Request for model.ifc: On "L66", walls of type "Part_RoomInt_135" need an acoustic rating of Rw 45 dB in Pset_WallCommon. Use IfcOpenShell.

First a look at what the model holds.

```python
import ifcopenshell
import ifcopenshell.util.element

model = ifcopenshell.open("model.ifc")
print(model.schema)
storey = next(s for s in model.by_type("IfcBuildingStorey") if s.Name == "L66")
walls = [e for e in ifcopenshell.util.element.get_decomposition(storey) if e.is_a("IfcWall")]
seen = {}
for e in walls:
    element_type = ifcopenshell.util.element.get_type(e)
    key = (element_type.Name if element_type != e and element_type else None, ifcopenshell.util.element.get_pset(e, "Pset_WallCommon", "AcousticRating"))
    seen[key] = seen.get(key, 0) + 1
for (name, value), count in sorted(seen.items(), key=str):
    print(count, "x", name, "|", value)
```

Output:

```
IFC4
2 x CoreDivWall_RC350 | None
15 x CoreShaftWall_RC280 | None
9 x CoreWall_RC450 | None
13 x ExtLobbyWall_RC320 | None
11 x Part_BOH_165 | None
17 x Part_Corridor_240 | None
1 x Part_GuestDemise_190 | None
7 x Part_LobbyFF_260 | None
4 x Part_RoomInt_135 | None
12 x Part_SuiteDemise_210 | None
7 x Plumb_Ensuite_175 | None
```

```python
import ifcopenshell
import ifcopenshell.api.pset
import ifcopenshell.util.element

model = ifcopenshell.open("model.ifc")

storey = next(s for s in model.by_type("IfcBuildingStorey") if s.Name == "L66")
walls = [e for e in ifcopenshell.util.element.get_decomposition(storey) if e.is_a("IfcWall")]

count = 0
for e in walls:
    element_type = ifcopenshell.util.element.get_type(e)
    if element_type in (None, e) or element_type.Name != "Part_RoomInt_135":
        continue
    found = ifcopenshell.util.element.get_pset(e, "Pset_WallCommon", should_inherit=False)
    if found:
        pset = model.by_id(found["id"])
        if len(ifcopenshell.util.element.get_elements_by_pset(pset)) > 1:
            pset = ifcopenshell.api.pset.unshare_pset(model, products=[e], pset=pset)[0]
    else:
        pset = ifcopenshell.api.pset.add_pset(model, product=e, name="Pset_WallCommon")
    ifcopenshell.api.pset.edit_pset(model, pset=pset, properties={"AcousticRating": "Rw 45 dB"})
    count += 1

print(count, "walls updated")

model.write("model_v2.ifc")
```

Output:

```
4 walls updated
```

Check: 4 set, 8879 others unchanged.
